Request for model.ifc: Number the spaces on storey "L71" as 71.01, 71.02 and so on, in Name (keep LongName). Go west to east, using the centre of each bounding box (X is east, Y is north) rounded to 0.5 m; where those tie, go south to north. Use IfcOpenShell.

First a look at what the model holds.

```python
import ifcopenshell
import ifcopenshell.util.element
import ifcopenshell.util.placement

model = ifcopenshell.open("model.ifc")
print(model.schema)
storey = next(s for s in model.by_type("IfcBuildingStorey") if s.Name == "L71")
spaces = [e for e in ifcopenshell.util.element.get_decomposition(storey) if e.is_a("IfcSpace")]
for e in sorted(spaces, key=lambda e: e.id()):
    origin = ifcopenshell.util.placement.get_local_placement(e.ObjectPlacement)[:3, 3]
    print(e.id(), e.Name, e.LongName, origin.round(2) + 0.0, sep=" | ")
```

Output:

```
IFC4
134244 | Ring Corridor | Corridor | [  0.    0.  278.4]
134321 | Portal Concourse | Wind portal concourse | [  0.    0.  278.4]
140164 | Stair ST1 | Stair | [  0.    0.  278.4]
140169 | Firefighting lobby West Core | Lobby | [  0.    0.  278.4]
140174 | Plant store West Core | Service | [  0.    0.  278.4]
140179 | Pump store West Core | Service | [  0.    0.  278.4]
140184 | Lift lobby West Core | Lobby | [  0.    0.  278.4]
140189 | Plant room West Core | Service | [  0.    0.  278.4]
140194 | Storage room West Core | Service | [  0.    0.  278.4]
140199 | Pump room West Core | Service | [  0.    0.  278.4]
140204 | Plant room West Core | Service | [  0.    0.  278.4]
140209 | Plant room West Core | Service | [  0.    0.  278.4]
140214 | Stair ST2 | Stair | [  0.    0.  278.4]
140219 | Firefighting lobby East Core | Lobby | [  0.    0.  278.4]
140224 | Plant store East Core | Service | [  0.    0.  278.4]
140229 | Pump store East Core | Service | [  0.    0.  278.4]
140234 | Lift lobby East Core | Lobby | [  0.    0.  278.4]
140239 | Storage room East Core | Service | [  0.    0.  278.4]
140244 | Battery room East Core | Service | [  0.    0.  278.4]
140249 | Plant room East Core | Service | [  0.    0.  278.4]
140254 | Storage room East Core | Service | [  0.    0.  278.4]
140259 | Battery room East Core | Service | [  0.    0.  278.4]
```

```python
import ifcopenshell
import ifcopenshell.geom
import ifcopenshell.util.element
import ifcopenshell.util.shape

model = ifcopenshell.open("model.ifc")
settings = ifcopenshell.geom.settings()
settings.set("use-world-coords", True)


def centre(element):
    shape = ifcopenshell.geom.create_shape(settings, element)
    return ifcopenshell.util.shape.get_bbox_centroid(shape.geometry)


storey = next(s for s in model.by_type("IfcBuildingStorey") if s.Name == "L71")
spaces = [e for e in ifcopenshell.util.element.get_decomposition(storey) if e.is_a("IfcSpace")]

# Insertion points can sit at a corner or the storey origin, so sort by the geometry (in metres).
centres = {e: centre(e) for e in spaces}
spaces.sort(key=lambda e: (round(centres[e][0] / 0.5), centres[e][1]))

for i, e in enumerate(spaces, start=1):
    number = f"71.{i:02d}"
    e.Name = number
    print(e.id(), number)

model.write("model_updated.ifc")
```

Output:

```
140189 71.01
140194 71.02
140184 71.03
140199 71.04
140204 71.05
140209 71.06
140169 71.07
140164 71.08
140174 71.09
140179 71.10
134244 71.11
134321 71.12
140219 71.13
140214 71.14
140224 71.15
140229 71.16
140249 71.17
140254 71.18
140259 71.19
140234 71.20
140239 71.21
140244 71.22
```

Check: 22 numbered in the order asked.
